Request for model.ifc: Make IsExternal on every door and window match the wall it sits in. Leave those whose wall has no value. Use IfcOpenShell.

First a look at what the model holds.

```python
import ifcopenshell
import ifcopenshell.util.element

model = ifcopenshell.open("model.ifc")
print(model.schema)
seen = {}
for e in model.by_type("IfcDoor") + model.by_type("IfcWindow"):
    if not e.FillsVoids:
        continue
    host = e.FillsVoids[0].RelatingOpeningElement.VoidsElements[0].RelatingBuildingElement
    own = ifcopenshell.util.element.get_pset(e, f"Pset_{e.is_a()[3:].removesuffix('StandardCase')}Common", "IsExternal")
    wall = ifcopenshell.util.element.get_pset(host, "Pset_WallCommon", "IsExternal")
    seen[e.is_a(), own, wall] = seen.get((e.is_a(), own, wall), 0) + 1
for (cls, own, wall), count in sorted(seen.items(), key=str):
    print(count, cls, "IsExternal:", own, "| host wall:", wall)
```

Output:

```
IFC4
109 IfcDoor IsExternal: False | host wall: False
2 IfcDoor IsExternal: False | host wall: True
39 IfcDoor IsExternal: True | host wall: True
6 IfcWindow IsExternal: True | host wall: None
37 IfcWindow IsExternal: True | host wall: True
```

```python
import ifcopenshell
import ifcopenshell.api.pset
import ifcopenshell.util.element

model = ifcopenshell.open("model.ifc")

count = 0
for ifc_class, pset_name in (("IfcDoor", "Pset_DoorCommon"), ("IfcWindow", "Pset_WindowCommon")):
    for e in model.by_type(ifc_class):
        if not e.FillsVoids:
            continue
        host = e.FillsVoids[0].RelatingOpeningElement.VoidsElements[0].RelatingBuildingElement
        external = ifcopenshell.util.element.get_pset(host, "Pset_WallCommon", "IsExternal")
        if external is None or ifcopenshell.util.element.get_pset(e, pset_name, "IsExternal") == external:
            continue
        pset = ifcopenshell.api.pset.add_pset(model, product=e, name=pset_name)
        ifcopenshell.api.pset.edit_pset(model, pset=pset, properties={"IsExternal": external})
        count += 1

print(count, "updated")

model.write("model-out.ifc")
```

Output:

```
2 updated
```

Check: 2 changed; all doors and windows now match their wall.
